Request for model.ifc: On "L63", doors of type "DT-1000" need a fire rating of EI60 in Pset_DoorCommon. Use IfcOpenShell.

First a look at what the model holds.

```python
import ifcopenshell
import ifcopenshell.util.element

model = ifcopenshell.open("model.ifc")
print(model.schema)
storey = next(s for s in model.by_type("IfcBuildingStorey") if s.Name == "L63")
doors = [e for e in ifcopenshell.util.element.get_decomposition(storey) if e.is_a("IfcDoor")]
seen = {}
for e in doors:
    element_type = ifcopenshell.util.element.get_type(e)
    key = (element_type.Name if element_type != e and element_type else None, ifcopenshell.util.element.get_pset(e, "Pset_DoorCommon", "FireRating"))
    seen[key] = seen.get(key, 0) + 1
for (name, value), count in sorted(seen.items(), key=str):
    print(count, "x", name, "|", value)
```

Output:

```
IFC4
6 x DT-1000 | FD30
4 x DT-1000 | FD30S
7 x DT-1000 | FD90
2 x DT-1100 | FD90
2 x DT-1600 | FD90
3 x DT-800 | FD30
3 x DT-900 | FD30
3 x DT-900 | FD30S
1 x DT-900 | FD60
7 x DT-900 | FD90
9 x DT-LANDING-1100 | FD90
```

```python
import ifcopenshell
import ifcopenshell.api.pset
import ifcopenshell.util.element

model = ifcopenshell.open("model.ifc")

storey = next(s for s in model.by_type("IfcBuildingStorey") if s.Name == "L63")
doors = [e for e in ifcopenshell.util.element.get_decomposition(storey) if e.is_a("IfcDoor")]

count = 0
for e in doors:
    element_type = ifcopenshell.util.element.get_type(e)
    if element_type in (None, e) or element_type.Name != "DT-1000":
        continue
    # add_pset returns the element's existing set when there is one.
    pset = ifcopenshell.api.pset.add_pset(model, product=e, name="Pset_DoorCommon")
    ifcopenshell.api.pset.edit_pset(model, pset=pset, properties={"FireRating": "EI60"})
    count += 1

print(count, "doors updated")

model.write("model_v2.ifc")
```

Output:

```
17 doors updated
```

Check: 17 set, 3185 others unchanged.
